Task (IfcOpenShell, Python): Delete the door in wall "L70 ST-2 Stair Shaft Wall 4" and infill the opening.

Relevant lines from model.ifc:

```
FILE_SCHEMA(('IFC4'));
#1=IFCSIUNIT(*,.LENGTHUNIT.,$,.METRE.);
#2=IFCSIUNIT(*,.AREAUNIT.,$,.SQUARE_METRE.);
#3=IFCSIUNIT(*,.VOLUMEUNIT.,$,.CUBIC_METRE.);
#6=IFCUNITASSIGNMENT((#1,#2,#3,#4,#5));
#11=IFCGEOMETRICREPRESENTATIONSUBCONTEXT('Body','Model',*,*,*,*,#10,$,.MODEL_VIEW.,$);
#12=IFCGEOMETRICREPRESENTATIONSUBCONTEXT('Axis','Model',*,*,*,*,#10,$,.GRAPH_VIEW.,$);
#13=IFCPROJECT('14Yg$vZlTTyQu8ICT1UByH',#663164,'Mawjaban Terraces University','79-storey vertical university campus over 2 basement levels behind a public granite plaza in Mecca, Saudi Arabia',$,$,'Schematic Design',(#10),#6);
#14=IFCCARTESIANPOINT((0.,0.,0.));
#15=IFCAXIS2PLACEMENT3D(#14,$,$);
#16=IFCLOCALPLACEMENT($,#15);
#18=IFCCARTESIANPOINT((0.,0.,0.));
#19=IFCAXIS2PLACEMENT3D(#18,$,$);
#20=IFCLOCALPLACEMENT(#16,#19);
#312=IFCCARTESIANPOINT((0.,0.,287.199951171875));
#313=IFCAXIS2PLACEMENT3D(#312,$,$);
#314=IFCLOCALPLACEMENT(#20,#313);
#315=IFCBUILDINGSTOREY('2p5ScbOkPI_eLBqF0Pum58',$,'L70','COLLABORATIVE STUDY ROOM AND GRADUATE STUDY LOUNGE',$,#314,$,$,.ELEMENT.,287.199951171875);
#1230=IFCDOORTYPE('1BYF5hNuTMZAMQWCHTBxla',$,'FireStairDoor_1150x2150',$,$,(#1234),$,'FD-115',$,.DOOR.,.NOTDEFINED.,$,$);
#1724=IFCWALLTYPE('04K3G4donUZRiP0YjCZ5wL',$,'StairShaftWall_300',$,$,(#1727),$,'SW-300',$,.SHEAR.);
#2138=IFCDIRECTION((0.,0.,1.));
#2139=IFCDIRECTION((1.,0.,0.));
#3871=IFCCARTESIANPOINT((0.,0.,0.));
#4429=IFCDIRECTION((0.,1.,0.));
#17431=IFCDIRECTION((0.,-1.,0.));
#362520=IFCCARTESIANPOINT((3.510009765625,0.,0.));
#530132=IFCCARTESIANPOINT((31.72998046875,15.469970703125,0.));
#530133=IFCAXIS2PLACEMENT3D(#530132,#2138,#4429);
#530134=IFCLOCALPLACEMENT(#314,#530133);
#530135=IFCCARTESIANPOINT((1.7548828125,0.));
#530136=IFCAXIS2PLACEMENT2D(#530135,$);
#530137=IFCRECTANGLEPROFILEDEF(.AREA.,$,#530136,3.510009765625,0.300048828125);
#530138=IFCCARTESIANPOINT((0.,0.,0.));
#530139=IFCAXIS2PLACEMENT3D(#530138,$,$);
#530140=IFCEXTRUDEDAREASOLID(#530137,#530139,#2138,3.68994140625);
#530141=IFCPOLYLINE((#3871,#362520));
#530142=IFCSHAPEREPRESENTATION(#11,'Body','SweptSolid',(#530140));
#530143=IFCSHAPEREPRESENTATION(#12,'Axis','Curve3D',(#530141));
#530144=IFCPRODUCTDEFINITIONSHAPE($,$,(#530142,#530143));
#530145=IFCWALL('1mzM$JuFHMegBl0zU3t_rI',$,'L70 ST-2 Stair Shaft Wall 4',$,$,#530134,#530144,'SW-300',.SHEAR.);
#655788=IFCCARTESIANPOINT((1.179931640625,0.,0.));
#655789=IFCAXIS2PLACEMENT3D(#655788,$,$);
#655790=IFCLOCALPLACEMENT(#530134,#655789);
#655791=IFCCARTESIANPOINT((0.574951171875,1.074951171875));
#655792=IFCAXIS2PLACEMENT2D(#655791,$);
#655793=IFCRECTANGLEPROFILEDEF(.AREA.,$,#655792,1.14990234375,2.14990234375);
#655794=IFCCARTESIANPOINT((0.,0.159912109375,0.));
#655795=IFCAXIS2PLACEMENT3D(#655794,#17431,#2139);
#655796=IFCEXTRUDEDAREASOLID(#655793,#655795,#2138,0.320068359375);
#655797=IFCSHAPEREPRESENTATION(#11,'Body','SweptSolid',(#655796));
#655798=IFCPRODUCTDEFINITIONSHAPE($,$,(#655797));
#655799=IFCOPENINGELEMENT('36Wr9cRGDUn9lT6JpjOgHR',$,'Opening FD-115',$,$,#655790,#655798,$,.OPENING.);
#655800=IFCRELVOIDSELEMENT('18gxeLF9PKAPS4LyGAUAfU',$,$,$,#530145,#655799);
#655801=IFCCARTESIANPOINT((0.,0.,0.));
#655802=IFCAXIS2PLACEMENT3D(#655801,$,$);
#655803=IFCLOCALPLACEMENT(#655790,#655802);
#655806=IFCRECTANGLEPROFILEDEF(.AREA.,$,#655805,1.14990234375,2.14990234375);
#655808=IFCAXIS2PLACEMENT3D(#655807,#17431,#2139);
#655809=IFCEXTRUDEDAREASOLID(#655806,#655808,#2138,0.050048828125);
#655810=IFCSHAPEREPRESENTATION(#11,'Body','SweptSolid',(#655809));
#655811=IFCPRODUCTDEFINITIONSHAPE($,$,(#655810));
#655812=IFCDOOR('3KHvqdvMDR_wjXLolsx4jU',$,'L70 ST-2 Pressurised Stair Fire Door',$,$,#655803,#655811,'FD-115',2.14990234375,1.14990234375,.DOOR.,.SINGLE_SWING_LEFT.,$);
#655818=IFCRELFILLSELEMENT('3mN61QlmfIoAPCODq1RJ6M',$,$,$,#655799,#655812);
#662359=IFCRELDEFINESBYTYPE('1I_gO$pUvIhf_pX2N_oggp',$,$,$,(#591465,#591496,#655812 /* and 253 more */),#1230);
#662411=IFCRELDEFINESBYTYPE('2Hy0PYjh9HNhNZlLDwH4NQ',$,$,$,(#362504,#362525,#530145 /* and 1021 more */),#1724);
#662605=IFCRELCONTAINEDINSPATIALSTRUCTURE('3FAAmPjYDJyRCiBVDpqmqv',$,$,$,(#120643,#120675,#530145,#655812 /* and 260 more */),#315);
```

```python
import ifcopenshell
import ifcopenshell.api.feature
import ifcopenshell.api.root
import ifcopenshell.geom
import ifcopenshell.util.shape

model = ifcopenshell.open("model.ifc")
settings = ifcopenshell.geom.settings()


def volume(element):
    """Net volume in cubic metres, openings subtracted."""
    shape = ifcopenshell.geom.create_shape(settings, element)
    return ifcopenshell.util.shape.get_volume(shape.geometry)


door = model.by_guid("3KHvqdvMDR_wjXLolsx4jU")
opening = door.FillsVoids[0].RelatingOpeningElement
wall = opening.VoidsElements[0].RelatingBuildingElement
before = volume(wall)

ifcopenshell.api.root.remove_product(model, product=door)
ifcopenshell.api.feature.remove_feature(model, feature=opening)

after = volume(wall)

print(f"wall volume {before:.3f} -> {after:.3f} m3")

model.write("model_updated.ifc")
```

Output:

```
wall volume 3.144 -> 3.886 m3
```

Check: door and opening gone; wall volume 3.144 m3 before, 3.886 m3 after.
